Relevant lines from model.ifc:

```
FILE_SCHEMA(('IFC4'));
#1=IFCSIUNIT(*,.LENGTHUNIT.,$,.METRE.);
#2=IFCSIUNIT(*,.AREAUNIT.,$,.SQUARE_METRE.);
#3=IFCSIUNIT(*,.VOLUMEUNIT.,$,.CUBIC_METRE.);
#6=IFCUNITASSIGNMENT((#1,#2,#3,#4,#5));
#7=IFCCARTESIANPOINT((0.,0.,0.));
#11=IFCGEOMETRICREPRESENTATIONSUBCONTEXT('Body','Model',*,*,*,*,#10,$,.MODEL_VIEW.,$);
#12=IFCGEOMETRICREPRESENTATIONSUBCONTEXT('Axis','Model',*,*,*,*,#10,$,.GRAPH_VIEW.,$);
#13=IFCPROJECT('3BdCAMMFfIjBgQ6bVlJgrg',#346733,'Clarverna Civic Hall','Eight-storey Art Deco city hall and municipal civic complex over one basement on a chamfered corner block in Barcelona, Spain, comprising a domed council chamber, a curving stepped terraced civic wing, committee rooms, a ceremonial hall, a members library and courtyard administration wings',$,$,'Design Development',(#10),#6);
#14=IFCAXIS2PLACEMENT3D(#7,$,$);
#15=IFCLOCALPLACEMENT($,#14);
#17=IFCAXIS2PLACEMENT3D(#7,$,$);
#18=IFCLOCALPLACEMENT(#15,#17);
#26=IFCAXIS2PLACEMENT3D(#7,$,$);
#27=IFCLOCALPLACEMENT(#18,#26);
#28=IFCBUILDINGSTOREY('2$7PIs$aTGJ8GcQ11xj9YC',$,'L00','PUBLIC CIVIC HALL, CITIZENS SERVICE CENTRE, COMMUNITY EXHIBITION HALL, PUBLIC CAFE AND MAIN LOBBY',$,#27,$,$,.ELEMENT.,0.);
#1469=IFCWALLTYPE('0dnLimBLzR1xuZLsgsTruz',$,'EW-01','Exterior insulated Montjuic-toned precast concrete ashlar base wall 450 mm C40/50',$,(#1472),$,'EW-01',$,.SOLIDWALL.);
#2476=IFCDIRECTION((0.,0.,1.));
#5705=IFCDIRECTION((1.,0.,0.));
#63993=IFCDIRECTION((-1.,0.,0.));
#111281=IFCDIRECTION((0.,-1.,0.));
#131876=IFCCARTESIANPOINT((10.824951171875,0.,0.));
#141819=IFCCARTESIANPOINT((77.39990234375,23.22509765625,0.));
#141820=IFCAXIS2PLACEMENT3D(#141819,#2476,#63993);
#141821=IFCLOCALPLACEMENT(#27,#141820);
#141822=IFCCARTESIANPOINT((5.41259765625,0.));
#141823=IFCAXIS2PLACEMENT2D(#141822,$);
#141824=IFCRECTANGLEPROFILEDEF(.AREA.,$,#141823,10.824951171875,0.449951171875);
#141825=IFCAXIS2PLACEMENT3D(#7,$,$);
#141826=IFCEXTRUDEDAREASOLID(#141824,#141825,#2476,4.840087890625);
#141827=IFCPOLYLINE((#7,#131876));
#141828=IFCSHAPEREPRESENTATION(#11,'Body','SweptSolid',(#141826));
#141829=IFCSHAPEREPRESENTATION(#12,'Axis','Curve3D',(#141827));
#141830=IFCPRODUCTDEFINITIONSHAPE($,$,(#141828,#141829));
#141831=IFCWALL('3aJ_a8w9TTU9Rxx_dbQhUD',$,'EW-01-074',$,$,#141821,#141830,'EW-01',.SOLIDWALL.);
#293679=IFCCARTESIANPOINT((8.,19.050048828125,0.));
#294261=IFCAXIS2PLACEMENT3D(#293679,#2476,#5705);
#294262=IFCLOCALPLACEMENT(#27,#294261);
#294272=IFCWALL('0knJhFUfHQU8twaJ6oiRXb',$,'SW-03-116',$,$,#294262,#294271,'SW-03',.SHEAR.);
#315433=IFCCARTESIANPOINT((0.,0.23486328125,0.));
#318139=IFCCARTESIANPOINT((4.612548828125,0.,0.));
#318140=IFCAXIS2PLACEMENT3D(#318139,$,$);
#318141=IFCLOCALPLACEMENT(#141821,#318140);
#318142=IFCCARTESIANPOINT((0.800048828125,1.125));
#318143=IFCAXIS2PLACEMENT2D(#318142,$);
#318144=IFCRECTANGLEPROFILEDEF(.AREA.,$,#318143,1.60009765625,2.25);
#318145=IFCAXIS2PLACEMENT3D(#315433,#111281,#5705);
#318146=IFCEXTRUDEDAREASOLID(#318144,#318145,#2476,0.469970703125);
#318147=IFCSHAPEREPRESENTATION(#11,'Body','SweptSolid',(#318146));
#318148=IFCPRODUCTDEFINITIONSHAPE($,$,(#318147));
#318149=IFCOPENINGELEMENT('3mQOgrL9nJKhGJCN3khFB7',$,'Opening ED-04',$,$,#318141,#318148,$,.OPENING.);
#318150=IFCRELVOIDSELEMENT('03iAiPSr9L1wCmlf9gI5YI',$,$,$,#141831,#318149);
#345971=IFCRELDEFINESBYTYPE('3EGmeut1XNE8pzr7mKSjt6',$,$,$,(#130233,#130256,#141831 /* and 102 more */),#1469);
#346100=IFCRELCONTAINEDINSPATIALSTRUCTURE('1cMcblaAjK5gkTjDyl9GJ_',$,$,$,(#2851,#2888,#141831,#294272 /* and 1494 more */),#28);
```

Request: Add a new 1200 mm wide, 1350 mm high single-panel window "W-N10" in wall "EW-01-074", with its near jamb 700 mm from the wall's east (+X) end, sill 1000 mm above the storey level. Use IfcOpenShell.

```python
import numpy as np
import ifcopenshell
import ifcopenshell.api.feature
import ifcopenshell.api.geometry
import ifcopenshell.api.root
import ifcopenshell.api.spatial
import ifcopenshell.geom
import ifcopenshell.util.element
import ifcopenshell.util.placement
import ifcopenshell.util.representation
import ifcopenshell.util.shape
import ifcopenshell.util.unit

model = ifcopenshell.open("model.ifc")
unit_scale = ifcopenshell.util.unit.calculate_unit_scale(model)
settings = ifcopenshell.geom.settings()


def volume(element):
    """Net volume in cubic metres, openings subtracted."""
    shape = ifcopenshell.geom.create_shape(settings, element)
    return ifcopenshell.util.shape.get_volume(shape.geometry)


wall = model.by_guid("3aJ_a8w9TTU9Rxx_dbQhUD")
storey = ifcopenshell.util.element.get_container(wall, ifc_class="IfcBuildingStorey")
context = ifcopenshell.util.representation.get_context(model, "Model", "Body", "MODEL_VIEW")
before = volume(wall)

width, height, from_end, sill = 1.2, 1.35, 0.7, 1  # metres

# The wall runs along its own X axis, and the end named is its -X end.
wall_shape = ifcopenshell.geom.create_shape(settings, wall)
x, y, z = ifcopenshell.util.shape.get_vertices(wall_shape.geometry).T
start = x.min() + from_end
face, thickness = float(y.min()), float(y.max() - y.min())
wall_matrix = ifcopenshell.util.placement.get_local_placement(wall.ObjectPlacement)
level = ifcopenshell.util.placement.get_local_placement(storey.ObjectPlacement)[2, 3]


def in_wall(x, y):
    """Placement at x, y metres in the wall's axes, at sill height."""
    matrix = wall_matrix.copy()
    matrix[:, 3] = wall_matrix @ np.array([x / unit_scale, y / unit_scale, 0.0, 1.0])
    matrix[2, 3] = level + sill / unit_scale
    return matrix


# Opening: a box that overshoots both wall faces by 50 mm.
opening = ifcopenshell.api.root.create_entity(model, ifc_class="IfcOpeningElement", predefined_type="OPENING")
box = ifcopenshell.api.geometry.add_wall_representation(
    model, context=context, length=width, height=height, thickness=thickness + 0.1
)
ifcopenshell.api.geometry.assign_representation(model, product=opening, representation=box)
ifcopenshell.api.geometry.edit_object_placement(model, product=opening, matrix=in_wall(start, face - 0.05), is_si=False)
ifcopenshell.api.feature.add_feature(model, feature=opening, element=wall)

window = ifcopenshell.api.root.create_entity(model, ifc_class="IfcWindow", name="W-N10", predefined_type="WINDOW")
window.OverallWidth, window.OverallHeight = width / unit_scale, height / unit_scale
window.PartitioningType = "SINGLE_PANEL"
body = ifcopenshell.api.geometry.add_window_representation(
    model,
    context=context,
    overall_width=window.OverallWidth,
    overall_height=window.OverallHeight,
    partition_type="SINGLE_PANEL",
)
ifcopenshell.api.geometry.assign_representation(model, product=window, representation=body)
ifcopenshell.api.spatial.assign_container(model, products=[window], relating_structure=storey)
ifcopenshell.api.feature.add_filling(model, opening=opening, element=window)

# Centre the window in the wall's thickness.
ifcopenshell.api.geometry.edit_object_placement(model, product=window, matrix=in_wall(start, face), is_si=False)
window_shape = ifcopenshell.geom.create_shape(settings, window)
depth = ifcopenshell.util.shape.get_vertices(window_shape.geometry)[:, 1]
offset = face + thickness / 2 - (depth.min() + depth.max()) / 2
ifcopenshell.api.geometry.edit_object_placement(model, product=window, matrix=in_wall(start, offset), is_si=False)

after = volume(wall)

print(f"wall volume {before:.3f} -> {after:.3f} m3")

model.write("model_rev.ifc")
```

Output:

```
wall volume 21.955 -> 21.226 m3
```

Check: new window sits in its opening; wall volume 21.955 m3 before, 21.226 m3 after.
